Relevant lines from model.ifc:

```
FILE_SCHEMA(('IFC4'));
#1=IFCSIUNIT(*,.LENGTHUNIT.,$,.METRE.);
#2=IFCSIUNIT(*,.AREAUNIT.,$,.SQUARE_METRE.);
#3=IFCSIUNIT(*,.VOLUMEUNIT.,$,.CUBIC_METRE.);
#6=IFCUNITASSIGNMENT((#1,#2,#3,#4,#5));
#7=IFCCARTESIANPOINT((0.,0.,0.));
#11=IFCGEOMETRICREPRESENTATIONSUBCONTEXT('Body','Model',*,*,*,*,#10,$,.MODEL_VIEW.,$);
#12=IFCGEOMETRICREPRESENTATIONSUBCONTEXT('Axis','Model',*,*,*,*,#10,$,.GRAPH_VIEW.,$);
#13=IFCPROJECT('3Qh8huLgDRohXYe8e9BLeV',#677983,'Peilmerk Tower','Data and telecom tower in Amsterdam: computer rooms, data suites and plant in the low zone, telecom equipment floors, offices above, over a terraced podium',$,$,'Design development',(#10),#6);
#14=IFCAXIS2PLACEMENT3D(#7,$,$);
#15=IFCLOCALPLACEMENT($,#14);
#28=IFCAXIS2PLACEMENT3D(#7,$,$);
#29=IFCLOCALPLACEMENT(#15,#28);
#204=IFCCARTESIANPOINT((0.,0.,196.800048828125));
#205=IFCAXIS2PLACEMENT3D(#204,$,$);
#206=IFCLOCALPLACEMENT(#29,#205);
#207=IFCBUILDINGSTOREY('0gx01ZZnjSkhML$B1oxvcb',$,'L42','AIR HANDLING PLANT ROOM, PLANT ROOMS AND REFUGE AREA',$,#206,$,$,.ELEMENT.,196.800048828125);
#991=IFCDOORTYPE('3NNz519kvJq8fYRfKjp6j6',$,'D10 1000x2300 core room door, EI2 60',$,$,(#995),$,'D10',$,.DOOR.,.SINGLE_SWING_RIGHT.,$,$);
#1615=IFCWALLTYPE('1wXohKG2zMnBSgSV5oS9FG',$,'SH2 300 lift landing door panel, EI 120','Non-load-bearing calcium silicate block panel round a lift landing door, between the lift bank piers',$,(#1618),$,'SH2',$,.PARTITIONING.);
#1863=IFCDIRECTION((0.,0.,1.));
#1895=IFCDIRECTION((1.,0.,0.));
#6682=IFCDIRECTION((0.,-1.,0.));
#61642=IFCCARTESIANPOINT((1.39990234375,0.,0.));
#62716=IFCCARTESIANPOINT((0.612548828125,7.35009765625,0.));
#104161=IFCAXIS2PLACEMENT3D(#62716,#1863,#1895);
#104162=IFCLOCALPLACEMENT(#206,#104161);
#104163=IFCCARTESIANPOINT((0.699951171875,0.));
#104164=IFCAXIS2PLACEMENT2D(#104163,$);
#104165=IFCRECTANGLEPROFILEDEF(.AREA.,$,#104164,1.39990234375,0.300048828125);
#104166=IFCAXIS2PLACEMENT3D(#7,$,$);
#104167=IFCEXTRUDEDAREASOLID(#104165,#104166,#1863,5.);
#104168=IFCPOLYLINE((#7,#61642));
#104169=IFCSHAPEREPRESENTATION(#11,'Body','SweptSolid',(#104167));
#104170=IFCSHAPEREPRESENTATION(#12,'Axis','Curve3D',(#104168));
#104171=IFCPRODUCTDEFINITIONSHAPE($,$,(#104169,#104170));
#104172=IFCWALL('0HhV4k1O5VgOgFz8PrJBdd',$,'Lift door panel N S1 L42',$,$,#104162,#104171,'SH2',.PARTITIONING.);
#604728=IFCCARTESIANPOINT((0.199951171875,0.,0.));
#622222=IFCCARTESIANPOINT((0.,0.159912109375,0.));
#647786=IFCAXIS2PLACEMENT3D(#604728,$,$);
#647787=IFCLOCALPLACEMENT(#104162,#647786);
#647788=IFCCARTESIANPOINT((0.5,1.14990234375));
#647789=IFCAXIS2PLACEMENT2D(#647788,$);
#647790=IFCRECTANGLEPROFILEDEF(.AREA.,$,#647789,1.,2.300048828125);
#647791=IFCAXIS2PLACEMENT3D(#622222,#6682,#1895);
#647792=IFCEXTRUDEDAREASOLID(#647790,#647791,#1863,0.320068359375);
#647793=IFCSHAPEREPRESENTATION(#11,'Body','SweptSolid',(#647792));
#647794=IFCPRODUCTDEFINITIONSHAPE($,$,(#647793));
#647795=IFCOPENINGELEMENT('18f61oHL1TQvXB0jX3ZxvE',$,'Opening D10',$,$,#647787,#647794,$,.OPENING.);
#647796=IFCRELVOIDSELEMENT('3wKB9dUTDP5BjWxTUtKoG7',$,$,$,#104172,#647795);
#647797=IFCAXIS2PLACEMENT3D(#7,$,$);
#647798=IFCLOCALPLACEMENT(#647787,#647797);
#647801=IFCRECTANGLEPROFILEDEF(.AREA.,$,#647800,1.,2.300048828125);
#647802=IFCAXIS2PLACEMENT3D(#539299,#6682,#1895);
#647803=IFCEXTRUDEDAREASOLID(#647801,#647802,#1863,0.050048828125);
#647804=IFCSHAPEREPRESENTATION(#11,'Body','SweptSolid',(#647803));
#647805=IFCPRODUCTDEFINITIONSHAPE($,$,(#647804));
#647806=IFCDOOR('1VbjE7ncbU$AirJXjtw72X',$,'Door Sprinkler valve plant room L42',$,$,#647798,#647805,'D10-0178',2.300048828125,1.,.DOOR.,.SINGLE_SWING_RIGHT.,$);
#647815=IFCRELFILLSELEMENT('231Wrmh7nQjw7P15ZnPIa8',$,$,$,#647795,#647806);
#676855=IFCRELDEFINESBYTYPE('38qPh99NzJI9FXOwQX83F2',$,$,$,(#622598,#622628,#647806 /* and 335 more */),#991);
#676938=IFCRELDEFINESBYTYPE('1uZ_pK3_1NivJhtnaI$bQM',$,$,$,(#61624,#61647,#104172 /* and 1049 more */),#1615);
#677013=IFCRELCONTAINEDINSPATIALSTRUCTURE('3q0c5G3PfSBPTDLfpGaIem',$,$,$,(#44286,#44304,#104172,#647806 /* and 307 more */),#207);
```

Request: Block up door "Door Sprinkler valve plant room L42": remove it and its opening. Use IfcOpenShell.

```python
import ifcopenshell
import ifcopenshell.api.feature
import ifcopenshell.api.root
import ifcopenshell.geom
import ifcopenshell.util.shape

model = ifcopenshell.open("model.ifc")
settings = ifcopenshell.geom.settings()


def volume(element):
    """Net volume in cubic metres, openings subtracted."""
    shape = ifcopenshell.geom.create_shape(settings, element)
    return ifcopenshell.util.shape.get_volume(shape.geometry)


door = model.by_id(647806)
opening = door.FillsVoids[0].RelatingOpeningElement
wall = opening.VoidsElements[0].RelatingBuildingElement
before = volume(wall)

ifcopenshell.api.root.remove_product(model, product=door)
ifcopenshell.api.feature.remove_feature(model, feature=opening)

after = volume(wall)

print(f"wall volume {before:.3f} -> {after:.3f} m3")

model.write("model_edited.ifc")
```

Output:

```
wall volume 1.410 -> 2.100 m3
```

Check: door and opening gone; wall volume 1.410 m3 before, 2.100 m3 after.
